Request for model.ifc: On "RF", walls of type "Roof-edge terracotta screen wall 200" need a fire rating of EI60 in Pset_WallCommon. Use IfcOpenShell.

First a look at what the model holds.

```python
import ifcopenshell
import ifcopenshell.util.element

model = ifcopenshell.open("model.ifc")
print(model.schema)
storey = next(s for s in model.by_type("IfcBuildingStorey") if s.Name == "RF")
walls = [e for e in ifcopenshell.util.element.get_decomposition(storey) if e.is_a("IfcWall")]
seen = {}
for e in walls:
    element_type = ifcopenshell.util.element.get_type(e)
    key = (element_type.Name if element_type != e and element_type else None, ifcopenshell.util.element.get_pset(e, "Pset_WallCommon", "FireRating"))
    seen[key] = seen.get(key, 0) + 1
for (name, value), count in sorted(seen.items(), key=str):
    print(count, "x", name, "|", value)
```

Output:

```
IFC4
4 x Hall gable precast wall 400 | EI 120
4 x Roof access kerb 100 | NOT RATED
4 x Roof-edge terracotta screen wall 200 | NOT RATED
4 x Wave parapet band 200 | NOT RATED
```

```python
import ifcopenshell
import ifcopenshell.api.pset
import ifcopenshell.util.element

model = ifcopenshell.open("model.ifc")

storey = next(s for s in model.by_type("IfcBuildingStorey") if s.Name == "RF")
walls = [e for e in ifcopenshell.util.element.get_decomposition(storey) if e.is_a("IfcWall")]

count = 0
for e in walls:
    element_type = ifcopenshell.util.element.get_type(e)
    if element_type in (None, e) or element_type.Name != "Roof-edge terracotta screen wall 200":
        continue
    # add_pset returns the element's existing set when there is one.
    pset = ifcopenshell.api.pset.add_pset(model, product=e, name="Pset_WallCommon")
    ifcopenshell.api.pset.edit_pset(model, pset=pset, properties={"FireRating": "EI60"})
    count += 1

print(count, "walls updated")

model.write("model_v2.ifc")
```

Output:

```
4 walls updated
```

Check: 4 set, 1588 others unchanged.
